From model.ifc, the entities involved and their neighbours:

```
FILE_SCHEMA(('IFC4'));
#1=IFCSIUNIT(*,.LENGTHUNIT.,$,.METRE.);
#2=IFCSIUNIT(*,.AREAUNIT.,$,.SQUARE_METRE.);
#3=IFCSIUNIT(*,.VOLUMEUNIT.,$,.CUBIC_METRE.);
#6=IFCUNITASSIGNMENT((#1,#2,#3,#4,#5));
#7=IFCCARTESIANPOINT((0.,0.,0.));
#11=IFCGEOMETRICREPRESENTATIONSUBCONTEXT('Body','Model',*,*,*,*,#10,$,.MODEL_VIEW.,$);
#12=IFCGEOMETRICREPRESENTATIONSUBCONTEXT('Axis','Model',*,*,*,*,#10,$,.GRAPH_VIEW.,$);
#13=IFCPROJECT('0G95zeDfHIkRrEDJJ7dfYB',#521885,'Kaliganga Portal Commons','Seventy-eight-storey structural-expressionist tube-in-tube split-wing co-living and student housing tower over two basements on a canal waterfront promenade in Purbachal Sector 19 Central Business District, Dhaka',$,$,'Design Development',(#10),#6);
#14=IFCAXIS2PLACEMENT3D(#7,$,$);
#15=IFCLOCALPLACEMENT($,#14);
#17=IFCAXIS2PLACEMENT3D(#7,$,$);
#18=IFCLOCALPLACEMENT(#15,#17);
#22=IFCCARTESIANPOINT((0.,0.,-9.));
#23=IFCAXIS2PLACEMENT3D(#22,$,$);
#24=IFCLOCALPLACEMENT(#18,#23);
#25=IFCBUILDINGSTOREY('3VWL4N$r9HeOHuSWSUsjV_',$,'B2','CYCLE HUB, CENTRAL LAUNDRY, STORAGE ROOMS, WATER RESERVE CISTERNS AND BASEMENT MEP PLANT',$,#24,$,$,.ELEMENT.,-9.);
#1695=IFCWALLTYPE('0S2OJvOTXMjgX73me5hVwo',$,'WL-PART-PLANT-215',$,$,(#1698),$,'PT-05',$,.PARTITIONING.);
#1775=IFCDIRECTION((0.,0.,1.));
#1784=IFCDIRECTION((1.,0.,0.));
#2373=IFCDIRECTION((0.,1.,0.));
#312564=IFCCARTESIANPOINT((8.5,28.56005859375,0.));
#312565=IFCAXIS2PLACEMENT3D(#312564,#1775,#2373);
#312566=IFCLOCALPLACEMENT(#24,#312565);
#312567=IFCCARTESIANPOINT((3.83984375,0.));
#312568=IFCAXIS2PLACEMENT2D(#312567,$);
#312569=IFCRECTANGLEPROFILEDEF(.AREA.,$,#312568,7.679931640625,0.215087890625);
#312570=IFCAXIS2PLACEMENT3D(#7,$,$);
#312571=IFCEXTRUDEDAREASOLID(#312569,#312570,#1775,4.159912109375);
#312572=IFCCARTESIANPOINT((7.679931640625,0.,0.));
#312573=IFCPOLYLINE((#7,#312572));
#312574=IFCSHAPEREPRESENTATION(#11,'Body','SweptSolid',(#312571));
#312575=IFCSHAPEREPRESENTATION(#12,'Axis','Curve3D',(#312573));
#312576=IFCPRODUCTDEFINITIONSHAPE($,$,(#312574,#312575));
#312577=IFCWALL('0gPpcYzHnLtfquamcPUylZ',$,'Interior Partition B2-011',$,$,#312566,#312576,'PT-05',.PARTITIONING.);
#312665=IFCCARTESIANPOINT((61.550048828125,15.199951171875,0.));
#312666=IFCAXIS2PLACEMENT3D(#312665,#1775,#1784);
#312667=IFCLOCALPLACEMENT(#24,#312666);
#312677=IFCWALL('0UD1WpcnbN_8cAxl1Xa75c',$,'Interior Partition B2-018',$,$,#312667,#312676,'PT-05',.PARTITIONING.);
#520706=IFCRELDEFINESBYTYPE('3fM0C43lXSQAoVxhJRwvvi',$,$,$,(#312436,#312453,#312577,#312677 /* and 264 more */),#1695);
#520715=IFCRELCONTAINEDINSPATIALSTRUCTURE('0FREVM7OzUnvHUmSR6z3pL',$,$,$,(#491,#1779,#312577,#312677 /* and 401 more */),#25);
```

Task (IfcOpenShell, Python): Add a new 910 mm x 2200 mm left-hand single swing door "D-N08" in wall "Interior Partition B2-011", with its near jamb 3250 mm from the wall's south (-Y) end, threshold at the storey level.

```python
import numpy as np
import ifcopenshell
import ifcopenshell.api.feature
import ifcopenshell.api.geometry
import ifcopenshell.api.root
import ifcopenshell.api.spatial
import ifcopenshell.geom
import ifcopenshell.util.element
import ifcopenshell.util.placement
import ifcopenshell.util.representation
import ifcopenshell.util.shape
import ifcopenshell.util.unit

model = ifcopenshell.open("model.ifc")
unit_scale = ifcopenshell.util.unit.calculate_unit_scale(model)
settings = ifcopenshell.geom.settings()


def volume(element):
    """Net volume in cubic metres, openings subtracted."""
    shape = ifcopenshell.geom.create_shape(settings, element)
    return ifcopenshell.util.shape.get_volume(shape.geometry)


wall = model.by_guid("0gPpcYzHnLtfquamcPUylZ")
storey = ifcopenshell.util.element.get_container(wall, ifc_class="IfcBuildingStorey")
context = ifcopenshell.util.representation.get_context(model, "Model", "Body", "MODEL_VIEW")
before = volume(wall)

width, height, from_end, sill = 0.91, 2.2, 3.25, 0.0  # metres

# The wall runs along its own X axis, and the end named is its -X end.
wall_shape = ifcopenshell.geom.create_shape(settings, wall)
x, y, z = ifcopenshell.util.shape.get_vertices(wall_shape.geometry).T
start = x.min() + from_end
face, thickness = float(y.min()), float(y.max() - y.min())
wall_matrix = ifcopenshell.util.placement.get_local_placement(wall.ObjectPlacement)
level = ifcopenshell.util.placement.get_local_placement(storey.ObjectPlacement)[2, 3]


def in_wall(x, y):
    """Placement at x, y metres in the wall's axes, at sill height."""
    matrix = wall_matrix.copy()
    matrix[:, 3] = wall_matrix @ np.array([x / unit_scale, y / unit_scale, 0.0, 1.0])
    matrix[2, 3] = level + sill / unit_scale
    return matrix


# Opening: a box that overshoots both wall faces by 50 mm.
opening = ifcopenshell.api.root.create_entity(model, ifc_class="IfcOpeningElement", predefined_type="OPENING")
box = ifcopenshell.api.geometry.add_wall_representation(
    model, context=context, length=width, height=height, thickness=thickness + 0.1
)
ifcopenshell.api.geometry.assign_representation(model, product=opening, representation=box)
ifcopenshell.api.geometry.edit_object_placement(model, product=opening, matrix=in_wall(start, face - 0.05), is_si=False)
ifcopenshell.api.feature.add_feature(model, feature=opening, element=wall)

door = ifcopenshell.api.root.create_entity(model, ifc_class="IfcDoor", name="D-N08", predefined_type="DOOR")
door.OverallWidth, door.OverallHeight = width / unit_scale, height / unit_scale
door.OperationType = "SINGLE_SWING_LEFT"
body = ifcopenshell.api.geometry.add_door_representation(
    model,
    context=context,
    overall_width=door.OverallWidth,
    overall_height=door.OverallHeight,
    operation_type="SINGLE_SWING_LEFT",
    lining_properties={"LiningDepth": thickness / unit_scale, "ThresholdDepth": thickness / unit_scale},
)
ifcopenshell.api.geometry.assign_representation(model, product=door, representation=body)
ifcopenshell.api.spatial.assign_container(model, products=[door], relating_structure=storey)
ifcopenshell.api.feature.add_filling(model, opening=opening, element=door)

# The lining spans the wall, so the door starts at the wall face.
ifcopenshell.api.geometry.edit_object_placement(model, product=door, matrix=in_wall(start, face), is_si=False)

after = volume(wall)

print(f"wall volume {before:.3f} -> {after:.3f} m3")

model.write("model-out.ifc")
```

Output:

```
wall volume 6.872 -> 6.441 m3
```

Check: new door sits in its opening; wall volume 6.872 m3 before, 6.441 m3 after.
